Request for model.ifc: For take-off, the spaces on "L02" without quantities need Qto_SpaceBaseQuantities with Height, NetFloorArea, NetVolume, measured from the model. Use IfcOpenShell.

First a look at what the model holds.

```python
import ifcopenshell
import ifcopenshell.util.element
import ifcopenshell.util.unit

model = ifcopenshell.open("model.ifc")
print(model.schema)
for unit_type in ("LENGTHUNIT", "AREAUNIT", "VOLUMEUNIT"):
    print(unit_type, ifcopenshell.util.unit.calculate_unit_scale(model, unit_type))
storey = next(s for s in model.by_type("IfcBuildingStorey") if s.Name == "L02")
spaces = [e for e in ifcopenshell.util.element.get_decomposition(storey) if e.is_a("IfcSpace")]
for e in sorted(spaces, key=lambda e: e.id()):
    print(e.id(), e.is_a(), e.Name, list(ifcopenshell.util.element.get_psets(e, qtos_only=True)), sep=" | ")
```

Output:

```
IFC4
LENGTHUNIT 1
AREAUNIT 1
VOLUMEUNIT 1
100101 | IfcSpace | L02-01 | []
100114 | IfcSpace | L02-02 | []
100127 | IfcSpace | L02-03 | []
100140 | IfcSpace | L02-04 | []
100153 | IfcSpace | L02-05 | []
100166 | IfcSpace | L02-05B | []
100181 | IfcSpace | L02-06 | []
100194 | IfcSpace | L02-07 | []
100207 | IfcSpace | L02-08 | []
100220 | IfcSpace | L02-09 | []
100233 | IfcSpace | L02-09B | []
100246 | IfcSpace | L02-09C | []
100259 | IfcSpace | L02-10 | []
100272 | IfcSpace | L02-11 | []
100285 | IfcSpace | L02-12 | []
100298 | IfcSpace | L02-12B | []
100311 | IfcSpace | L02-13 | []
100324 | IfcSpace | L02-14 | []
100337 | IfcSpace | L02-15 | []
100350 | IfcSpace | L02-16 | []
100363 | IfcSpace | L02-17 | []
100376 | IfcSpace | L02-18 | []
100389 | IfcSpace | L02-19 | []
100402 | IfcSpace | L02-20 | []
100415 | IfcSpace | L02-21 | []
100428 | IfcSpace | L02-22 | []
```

```python
import ifcopenshell
import ifcopenshell.api.pset
import ifcopenshell.geom
import ifcopenshell.util.element
import ifcopenshell.util.shape
import ifcopenshell.util.unit

model = ifcopenshell.open("model.ifc")
unit_scale = ifcopenshell.util.unit.calculate_unit_scale(model)
area_scale = ifcopenshell.util.unit.calculate_unit_scale(model, "AREAUNIT")
volume_scale = ifcopenshell.util.unit.calculate_unit_scale(model, "VOLUMEUNIT")
settings = ifcopenshell.geom.settings()

storey = next(s for s in model.by_type("IfcBuildingStorey") if s.Name == "L02")
spaces = [e for e in ifcopenshell.util.element.get_decomposition(storey) if e.is_a("IfcSpace")]

for e in sorted(spaces, key=lambda e: e.id()):
    if ifcopenshell.util.element.get_psets(e, qtos_only=True, should_inherit=False):
        continue
    # Geometry comes back in metres, in the element's own axes.
    shape = ifcopenshell.geom.create_shape(settings, e)
    values = {
        "Height": ifcopenshell.util.shape.get_z(shape.geometry) / unit_scale,
        "NetFloorArea": ifcopenshell.util.shape.get_footprint_area(shape.geometry) / area_scale,
        "NetVolume": ifcopenshell.util.shape.get_volume(shape.geometry) / volume_scale,
    }
    qto = ifcopenshell.api.pset.add_qto(model, product=e, name="Qto_SpaceBaseQuantities")
    ifcopenshell.api.pset.edit_qto(model, qto=qto, properties=values)
    print(e.id(), {k: round(v, 3) for k, v in values.items()})

model.write("model_rev.ifc")
```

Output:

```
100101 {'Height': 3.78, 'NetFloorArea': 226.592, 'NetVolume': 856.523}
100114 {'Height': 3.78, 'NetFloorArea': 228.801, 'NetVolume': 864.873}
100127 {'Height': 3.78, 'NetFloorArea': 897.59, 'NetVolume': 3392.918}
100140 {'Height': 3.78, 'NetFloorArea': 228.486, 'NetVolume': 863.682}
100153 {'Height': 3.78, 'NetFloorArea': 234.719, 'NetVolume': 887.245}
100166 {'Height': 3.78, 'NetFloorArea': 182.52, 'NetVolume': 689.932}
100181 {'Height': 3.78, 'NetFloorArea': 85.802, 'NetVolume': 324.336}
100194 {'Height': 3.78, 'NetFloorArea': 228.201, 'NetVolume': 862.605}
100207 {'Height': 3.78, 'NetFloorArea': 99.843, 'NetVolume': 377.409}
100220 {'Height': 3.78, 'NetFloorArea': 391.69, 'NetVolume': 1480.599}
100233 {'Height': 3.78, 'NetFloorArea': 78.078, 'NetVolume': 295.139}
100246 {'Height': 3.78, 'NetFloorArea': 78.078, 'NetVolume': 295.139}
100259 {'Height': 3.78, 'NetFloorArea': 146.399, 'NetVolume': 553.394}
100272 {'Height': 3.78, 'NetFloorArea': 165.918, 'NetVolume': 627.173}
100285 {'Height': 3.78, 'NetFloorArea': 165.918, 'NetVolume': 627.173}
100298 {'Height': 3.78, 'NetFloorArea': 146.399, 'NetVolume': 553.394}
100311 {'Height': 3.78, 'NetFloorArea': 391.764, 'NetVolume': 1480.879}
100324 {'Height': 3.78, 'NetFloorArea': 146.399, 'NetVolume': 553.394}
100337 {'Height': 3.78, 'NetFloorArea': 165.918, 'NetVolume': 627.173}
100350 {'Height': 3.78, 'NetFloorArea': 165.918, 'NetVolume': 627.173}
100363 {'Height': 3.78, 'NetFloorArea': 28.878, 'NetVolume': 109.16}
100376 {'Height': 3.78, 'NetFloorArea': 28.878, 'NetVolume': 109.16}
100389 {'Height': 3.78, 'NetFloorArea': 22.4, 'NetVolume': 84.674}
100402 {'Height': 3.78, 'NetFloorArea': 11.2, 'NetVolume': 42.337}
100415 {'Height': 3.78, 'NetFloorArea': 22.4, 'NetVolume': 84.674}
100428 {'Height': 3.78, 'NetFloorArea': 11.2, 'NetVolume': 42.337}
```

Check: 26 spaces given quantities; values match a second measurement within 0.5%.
